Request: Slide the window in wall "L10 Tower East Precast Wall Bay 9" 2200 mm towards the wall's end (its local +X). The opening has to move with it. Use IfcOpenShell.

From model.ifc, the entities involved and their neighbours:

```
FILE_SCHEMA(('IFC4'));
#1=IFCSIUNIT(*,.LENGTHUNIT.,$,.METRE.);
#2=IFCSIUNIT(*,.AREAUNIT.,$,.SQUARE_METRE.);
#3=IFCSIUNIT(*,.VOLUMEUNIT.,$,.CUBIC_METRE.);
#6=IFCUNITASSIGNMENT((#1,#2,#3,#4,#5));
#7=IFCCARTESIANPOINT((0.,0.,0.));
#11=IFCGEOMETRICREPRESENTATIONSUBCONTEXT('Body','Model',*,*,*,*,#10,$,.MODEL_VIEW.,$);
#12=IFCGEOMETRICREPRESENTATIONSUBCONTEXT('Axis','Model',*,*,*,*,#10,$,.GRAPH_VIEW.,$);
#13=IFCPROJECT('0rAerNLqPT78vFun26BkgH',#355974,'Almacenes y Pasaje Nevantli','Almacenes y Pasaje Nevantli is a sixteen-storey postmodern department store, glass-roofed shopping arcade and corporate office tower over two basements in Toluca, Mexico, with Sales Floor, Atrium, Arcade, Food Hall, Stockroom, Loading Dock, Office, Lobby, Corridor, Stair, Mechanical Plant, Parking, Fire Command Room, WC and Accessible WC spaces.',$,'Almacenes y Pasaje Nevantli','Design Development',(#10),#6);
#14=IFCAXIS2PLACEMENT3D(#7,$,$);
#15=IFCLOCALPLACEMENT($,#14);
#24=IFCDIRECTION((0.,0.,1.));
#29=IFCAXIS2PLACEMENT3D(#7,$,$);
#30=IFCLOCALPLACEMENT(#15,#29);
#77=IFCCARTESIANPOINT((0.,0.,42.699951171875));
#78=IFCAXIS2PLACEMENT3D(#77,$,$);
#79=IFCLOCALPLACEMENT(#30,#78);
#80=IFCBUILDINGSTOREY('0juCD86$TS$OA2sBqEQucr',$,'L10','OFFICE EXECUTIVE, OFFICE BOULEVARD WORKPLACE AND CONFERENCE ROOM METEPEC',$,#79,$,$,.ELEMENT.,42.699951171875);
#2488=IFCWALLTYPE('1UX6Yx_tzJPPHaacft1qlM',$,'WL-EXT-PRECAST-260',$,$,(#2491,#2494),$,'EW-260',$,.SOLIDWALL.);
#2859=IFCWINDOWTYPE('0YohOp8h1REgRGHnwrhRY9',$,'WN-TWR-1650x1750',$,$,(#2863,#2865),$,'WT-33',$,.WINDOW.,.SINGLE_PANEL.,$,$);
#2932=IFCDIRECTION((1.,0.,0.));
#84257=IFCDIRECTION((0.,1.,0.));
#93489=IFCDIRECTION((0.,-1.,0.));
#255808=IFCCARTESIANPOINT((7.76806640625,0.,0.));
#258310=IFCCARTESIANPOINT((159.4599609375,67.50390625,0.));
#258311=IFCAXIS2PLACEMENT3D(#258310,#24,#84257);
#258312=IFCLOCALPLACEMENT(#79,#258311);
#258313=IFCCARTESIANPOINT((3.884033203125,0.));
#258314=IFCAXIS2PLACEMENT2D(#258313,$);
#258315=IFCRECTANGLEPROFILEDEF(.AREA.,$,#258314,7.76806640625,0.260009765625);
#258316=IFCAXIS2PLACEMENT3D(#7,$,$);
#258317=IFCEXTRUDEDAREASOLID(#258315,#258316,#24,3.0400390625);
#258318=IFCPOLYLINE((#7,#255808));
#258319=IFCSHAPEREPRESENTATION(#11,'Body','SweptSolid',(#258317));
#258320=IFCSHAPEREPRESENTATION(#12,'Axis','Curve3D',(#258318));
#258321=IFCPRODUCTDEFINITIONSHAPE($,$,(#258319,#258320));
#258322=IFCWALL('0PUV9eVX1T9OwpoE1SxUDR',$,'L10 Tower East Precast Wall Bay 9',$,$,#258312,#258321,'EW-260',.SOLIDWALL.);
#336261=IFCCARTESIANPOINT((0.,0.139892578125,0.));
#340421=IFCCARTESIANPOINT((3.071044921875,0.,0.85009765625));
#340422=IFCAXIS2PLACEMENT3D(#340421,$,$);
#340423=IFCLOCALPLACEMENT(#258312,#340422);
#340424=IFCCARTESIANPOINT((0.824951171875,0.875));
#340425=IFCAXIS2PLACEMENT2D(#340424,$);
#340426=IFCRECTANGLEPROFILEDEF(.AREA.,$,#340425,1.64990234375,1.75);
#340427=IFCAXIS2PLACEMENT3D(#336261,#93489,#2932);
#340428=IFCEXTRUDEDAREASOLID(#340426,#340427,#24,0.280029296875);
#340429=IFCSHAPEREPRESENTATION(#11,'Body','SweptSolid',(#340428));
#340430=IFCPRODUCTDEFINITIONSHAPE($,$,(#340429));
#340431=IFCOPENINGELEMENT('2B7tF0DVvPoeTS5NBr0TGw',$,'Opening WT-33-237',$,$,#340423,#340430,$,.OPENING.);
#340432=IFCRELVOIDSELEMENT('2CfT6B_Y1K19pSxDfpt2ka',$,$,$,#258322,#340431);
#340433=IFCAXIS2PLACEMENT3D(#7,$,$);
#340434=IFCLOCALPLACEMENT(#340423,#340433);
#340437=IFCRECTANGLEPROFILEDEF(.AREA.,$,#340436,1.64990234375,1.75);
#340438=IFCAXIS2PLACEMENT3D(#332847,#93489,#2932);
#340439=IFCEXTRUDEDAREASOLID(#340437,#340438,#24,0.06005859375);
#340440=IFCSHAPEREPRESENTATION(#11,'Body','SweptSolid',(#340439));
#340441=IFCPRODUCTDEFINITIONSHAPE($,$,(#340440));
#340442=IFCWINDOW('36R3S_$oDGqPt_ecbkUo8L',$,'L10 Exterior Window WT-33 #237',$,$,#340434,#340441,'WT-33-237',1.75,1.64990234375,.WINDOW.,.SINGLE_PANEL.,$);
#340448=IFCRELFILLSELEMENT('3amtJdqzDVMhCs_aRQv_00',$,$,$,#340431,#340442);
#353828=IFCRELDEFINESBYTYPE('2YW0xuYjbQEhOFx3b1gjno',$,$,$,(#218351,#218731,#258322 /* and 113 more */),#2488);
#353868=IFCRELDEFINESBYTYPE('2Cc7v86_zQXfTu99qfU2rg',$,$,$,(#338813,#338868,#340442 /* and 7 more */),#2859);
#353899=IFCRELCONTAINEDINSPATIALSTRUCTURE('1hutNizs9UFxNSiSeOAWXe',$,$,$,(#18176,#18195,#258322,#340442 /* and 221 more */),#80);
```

```python
import ifcopenshell
import ifcopenshell.api.geometry
import ifcopenshell.util.placement
import ifcopenshell.util.unit

model = ifcopenshell.open("model.ifc")
unit_scale = ifcopenshell.util.unit.calculate_unit_scale(model)

window = model.by_guid("36R3S_$oDGqPt_ecbkUo8L")
opening = window.FillsVoids[0].RelatingOpeningElement
wall = opening.VoidsElements[0].RelatingBuildingElement

wall_matrix = ifcopenshell.util.placement.get_local_placement(wall.ObjectPlacement)
shift = wall_matrix[:3, 0] * 2.2 / unit_scale
before = ifcopenshell.util.placement.get_local_placement(window.ObjectPlacement)[:3, 3].copy()

# The window is placed relative to its opening, so it follows when the opening moves.
matrix = ifcopenshell.util.placement.get_local_placement(opening.ObjectPlacement)
matrix[:3, 3] += shift
ifcopenshell.api.geometry.edit_object_placement(
    model, product=opening, matrix=matrix, is_si=False, should_transform_children=True
)

after = ifcopenshell.util.placement.get_local_placement(window.ObjectPlacement)[:3, 3]
print("window moved by", (after - before).round(3) + 0.0)

model.write("model_rev.ifc")
```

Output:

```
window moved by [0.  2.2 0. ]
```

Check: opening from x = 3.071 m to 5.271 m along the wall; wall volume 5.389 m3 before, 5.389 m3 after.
